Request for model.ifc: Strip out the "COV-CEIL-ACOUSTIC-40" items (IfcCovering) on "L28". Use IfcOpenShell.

First a look at what the model holds.

```python
import ifcopenshell
import ifcopenshell.util.element

model = ifcopenshell.open("model.ifc")
print(model.schema)
storey = next(s for s in model.by_type("IfcBuildingStorey") if s.Name == "L28")
coverings = [e for e in ifcopenshell.util.element.get_decomposition(storey) if e.is_a("IfcCovering")]
seen = {}
for e in coverings:
    element_type = ifcopenshell.util.element.get_type(e)
    name = element_type.Name if element_type not in (None, e) else None
    seen[name] = seen.get(name, 0) + 1
for name, count in sorted(seen.items(), key=str):
    print(count, "x", name)
```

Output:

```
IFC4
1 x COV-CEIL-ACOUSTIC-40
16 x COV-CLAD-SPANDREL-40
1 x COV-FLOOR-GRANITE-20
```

```python
import ifcopenshell
import ifcopenshell.api.root
import ifcopenshell.util.element

model = ifcopenshell.open("model.ifc")

storey = next(s for s in model.by_type("IfcBuildingStorey") if s.Name == "L28")
coverings = [e for e in ifcopenshell.util.element.get_decomposition(storey) if e.is_a("IfcCovering")]
targets = [e for e in coverings if (t := ifcopenshell.util.element.get_type(e)) not in (None, e) and t.Name == "COV-CEIL-ACOUSTIC-40"]

for e in targets:
    ifcopenshell.api.root.remove_product(model, product=e)
print(len(targets), "removed")

model.write("model-out.ifc")
```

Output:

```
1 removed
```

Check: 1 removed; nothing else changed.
